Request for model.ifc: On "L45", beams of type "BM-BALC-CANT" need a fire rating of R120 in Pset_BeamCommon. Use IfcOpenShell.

First a look at what the model holds.

```python
import ifcopenshell
import ifcopenshell.util.element

model = ifcopenshell.open("model.ifc")
print(model.schema)
storey = next(s for s in model.by_type("IfcBuildingStorey") if s.Name == "L45")
beams = [e for e in ifcopenshell.util.element.get_decomposition(storey) if e.is_a("IfcBeam")]
seen = {}
for e in beams:
    element_type = ifcopenshell.util.element.get_type(e)
    key = (element_type.Name if element_type != e and element_type else None, ifcopenshell.util.element.get_pset(e, "Pset_BeamCommon", "FireRating"))
    seen[key] = seen.get(key, 0) + 1
for (name, value), count in sorted(seen.items(), key=str):
    print(count, "x", name, "|", value)
```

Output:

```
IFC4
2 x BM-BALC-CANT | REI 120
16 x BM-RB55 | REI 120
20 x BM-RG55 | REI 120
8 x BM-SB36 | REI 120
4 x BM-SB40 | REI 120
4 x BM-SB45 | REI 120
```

```python
import ifcopenshell
import ifcopenshell.api.pset
import ifcopenshell.util.element

model = ifcopenshell.open("model.ifc")

storey = next(s for s in model.by_type("IfcBuildingStorey") if s.Name == "L45")
beams = [e for e in ifcopenshell.util.element.get_decomposition(storey) if e.is_a("IfcBeam")]

count = 0
for e in beams:
    element_type = ifcopenshell.util.element.get_type(e)
    if element_type in (None, e) or element_type.Name != "BM-BALC-CANT":
        continue
    found = ifcopenshell.util.element.get_pset(e, "Pset_BeamCommon", should_inherit=False)
    if found:
        pset = model.by_id(found["id"])
        if len(ifcopenshell.util.element.get_elements_by_pset(pset)) > 1:
            pset = ifcopenshell.api.pset.unshare_pset(model, products=[e], pset=pset)[0]
    else:
        pset = ifcopenshell.api.pset.add_pset(model, product=e, name="Pset_BeamCommon")
    ifcopenshell.api.pset.edit_pset(model, pset=pset, properties={"FireRating": "R120"})
    count += 1

print(count, "beams updated")

model.write("model-out.ifc")
```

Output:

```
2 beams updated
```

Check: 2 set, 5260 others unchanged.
